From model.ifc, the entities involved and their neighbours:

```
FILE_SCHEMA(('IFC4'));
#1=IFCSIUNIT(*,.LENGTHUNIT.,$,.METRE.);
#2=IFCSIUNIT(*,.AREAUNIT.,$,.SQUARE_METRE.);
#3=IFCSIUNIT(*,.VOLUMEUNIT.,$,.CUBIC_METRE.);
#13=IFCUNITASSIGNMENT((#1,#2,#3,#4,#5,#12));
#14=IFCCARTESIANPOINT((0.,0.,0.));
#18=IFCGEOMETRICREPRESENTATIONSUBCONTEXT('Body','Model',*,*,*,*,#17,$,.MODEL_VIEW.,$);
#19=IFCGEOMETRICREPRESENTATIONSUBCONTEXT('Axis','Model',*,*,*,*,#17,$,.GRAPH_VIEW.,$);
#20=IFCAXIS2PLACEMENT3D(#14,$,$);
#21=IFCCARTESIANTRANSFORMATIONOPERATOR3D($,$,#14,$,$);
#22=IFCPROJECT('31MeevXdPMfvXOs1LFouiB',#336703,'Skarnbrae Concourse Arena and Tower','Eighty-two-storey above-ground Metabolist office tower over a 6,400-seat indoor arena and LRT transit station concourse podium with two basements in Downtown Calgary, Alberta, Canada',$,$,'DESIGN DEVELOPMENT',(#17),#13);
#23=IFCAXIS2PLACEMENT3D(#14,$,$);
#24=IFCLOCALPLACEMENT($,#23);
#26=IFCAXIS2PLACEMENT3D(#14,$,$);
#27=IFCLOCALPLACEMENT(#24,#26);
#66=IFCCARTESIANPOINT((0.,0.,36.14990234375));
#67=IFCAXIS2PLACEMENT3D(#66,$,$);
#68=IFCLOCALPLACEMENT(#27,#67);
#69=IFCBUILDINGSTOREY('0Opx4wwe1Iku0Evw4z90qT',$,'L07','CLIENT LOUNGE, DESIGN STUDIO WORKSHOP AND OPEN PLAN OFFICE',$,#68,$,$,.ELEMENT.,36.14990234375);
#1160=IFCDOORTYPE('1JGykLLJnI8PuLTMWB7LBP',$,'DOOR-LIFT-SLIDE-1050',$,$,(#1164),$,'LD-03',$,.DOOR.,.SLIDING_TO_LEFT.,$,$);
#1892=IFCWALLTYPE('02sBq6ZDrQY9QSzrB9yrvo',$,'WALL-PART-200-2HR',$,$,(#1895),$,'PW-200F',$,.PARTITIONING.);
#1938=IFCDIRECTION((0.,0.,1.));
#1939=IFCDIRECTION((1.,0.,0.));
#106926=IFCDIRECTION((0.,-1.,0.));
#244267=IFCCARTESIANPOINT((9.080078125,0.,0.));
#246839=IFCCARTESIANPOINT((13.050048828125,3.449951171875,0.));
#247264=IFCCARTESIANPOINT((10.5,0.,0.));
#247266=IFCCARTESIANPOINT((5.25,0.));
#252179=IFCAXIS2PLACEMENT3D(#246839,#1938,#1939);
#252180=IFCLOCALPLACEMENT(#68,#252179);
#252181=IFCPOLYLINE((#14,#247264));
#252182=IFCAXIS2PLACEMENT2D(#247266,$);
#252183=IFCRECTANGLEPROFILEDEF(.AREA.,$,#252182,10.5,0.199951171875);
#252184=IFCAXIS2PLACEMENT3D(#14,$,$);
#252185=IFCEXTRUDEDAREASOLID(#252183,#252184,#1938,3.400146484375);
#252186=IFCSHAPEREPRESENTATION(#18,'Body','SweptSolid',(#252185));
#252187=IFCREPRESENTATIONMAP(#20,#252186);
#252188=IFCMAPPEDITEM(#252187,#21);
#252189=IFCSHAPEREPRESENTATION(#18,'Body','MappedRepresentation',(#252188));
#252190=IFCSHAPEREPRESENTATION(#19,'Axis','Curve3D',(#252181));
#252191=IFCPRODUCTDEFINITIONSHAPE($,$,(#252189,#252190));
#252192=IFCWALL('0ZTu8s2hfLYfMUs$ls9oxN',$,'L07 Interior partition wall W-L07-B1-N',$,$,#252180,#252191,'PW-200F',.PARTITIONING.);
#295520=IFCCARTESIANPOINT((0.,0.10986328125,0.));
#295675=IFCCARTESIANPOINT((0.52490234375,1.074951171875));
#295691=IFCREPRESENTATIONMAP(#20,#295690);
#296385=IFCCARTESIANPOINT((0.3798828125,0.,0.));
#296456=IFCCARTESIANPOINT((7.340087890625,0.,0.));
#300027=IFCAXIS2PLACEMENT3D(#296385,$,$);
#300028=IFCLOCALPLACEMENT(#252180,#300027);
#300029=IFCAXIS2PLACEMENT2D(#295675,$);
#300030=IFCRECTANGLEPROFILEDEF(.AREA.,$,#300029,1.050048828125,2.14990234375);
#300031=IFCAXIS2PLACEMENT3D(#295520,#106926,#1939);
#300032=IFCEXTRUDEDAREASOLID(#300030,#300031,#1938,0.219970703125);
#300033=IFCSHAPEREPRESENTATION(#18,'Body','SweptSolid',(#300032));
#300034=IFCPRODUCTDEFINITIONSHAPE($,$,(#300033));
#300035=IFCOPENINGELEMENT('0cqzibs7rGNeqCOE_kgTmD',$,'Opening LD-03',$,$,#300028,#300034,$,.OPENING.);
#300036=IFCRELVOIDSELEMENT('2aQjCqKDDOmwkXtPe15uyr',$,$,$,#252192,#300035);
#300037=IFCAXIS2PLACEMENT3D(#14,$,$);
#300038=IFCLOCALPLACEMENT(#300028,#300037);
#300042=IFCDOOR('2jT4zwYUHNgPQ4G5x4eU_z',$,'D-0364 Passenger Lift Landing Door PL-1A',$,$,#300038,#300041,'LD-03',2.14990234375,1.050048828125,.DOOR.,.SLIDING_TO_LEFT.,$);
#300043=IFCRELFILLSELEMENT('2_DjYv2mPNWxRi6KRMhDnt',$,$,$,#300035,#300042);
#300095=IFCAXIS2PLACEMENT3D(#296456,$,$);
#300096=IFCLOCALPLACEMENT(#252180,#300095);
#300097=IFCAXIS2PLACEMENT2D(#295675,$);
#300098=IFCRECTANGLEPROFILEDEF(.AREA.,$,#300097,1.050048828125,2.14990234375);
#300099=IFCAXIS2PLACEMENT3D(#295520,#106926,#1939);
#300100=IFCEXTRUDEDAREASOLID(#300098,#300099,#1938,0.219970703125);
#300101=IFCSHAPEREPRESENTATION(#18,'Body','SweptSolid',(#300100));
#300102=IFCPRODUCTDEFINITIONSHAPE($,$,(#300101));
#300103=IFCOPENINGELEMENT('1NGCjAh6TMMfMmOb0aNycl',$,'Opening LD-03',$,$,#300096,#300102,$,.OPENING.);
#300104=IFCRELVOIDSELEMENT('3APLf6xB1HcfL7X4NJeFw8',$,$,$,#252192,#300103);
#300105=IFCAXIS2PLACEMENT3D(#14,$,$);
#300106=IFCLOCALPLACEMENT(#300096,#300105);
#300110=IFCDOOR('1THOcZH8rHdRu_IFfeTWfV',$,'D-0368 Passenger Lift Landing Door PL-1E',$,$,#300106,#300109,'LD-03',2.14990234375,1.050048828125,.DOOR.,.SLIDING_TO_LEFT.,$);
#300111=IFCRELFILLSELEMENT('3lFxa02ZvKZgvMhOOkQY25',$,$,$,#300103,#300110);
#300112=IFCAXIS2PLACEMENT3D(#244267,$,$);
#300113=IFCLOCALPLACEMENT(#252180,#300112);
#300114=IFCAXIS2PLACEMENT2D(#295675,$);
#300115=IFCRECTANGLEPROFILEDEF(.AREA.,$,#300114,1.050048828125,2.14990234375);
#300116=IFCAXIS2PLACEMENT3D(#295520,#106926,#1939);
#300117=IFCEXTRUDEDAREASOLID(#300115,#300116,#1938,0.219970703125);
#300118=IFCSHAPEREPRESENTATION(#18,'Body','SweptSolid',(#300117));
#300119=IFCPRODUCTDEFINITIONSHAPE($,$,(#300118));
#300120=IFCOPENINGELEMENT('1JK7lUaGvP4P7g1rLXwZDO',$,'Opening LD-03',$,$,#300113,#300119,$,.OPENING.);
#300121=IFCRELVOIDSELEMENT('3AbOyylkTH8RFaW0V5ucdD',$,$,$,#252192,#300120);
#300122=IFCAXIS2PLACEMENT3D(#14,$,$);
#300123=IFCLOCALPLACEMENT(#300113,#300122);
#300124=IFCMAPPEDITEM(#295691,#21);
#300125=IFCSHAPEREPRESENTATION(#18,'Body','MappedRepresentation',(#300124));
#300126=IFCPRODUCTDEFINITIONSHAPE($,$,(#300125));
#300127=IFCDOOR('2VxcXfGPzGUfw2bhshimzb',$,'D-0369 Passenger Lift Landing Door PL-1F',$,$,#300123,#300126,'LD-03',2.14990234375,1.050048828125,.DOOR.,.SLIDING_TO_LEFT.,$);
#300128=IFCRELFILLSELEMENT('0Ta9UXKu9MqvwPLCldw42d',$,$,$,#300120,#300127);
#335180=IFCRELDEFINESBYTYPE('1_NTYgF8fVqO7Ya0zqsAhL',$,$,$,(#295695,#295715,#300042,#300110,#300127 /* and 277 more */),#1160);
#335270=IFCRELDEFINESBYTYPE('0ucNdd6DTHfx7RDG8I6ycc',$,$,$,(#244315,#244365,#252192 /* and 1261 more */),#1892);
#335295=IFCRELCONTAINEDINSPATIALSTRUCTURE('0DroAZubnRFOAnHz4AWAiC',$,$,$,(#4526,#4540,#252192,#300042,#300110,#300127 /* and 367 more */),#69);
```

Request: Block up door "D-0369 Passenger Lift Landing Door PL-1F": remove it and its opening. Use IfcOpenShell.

```python
import ifcopenshell
import ifcopenshell.api.feature
import ifcopenshell.api.root
import ifcopenshell.geom
import ifcopenshell.util.shape

model = ifcopenshell.open("model.ifc")
settings = ifcopenshell.geom.settings()


def volume(element):
    """Net volume in cubic metres, openings subtracted."""
    shape = ifcopenshell.geom.create_shape(settings, element)
    return ifcopenshell.util.shape.get_volume(shape.geometry)


door = model.by_guid("2VxcXfGPzGUfw2bhshimzb")
opening = door.FillsVoids[0].RelatingOpeningElement
wall = opening.VoidsElements[0].RelatingBuildingElement
before = volume(wall)

ifcopenshell.api.root.remove_product(model, product=door)
ifcopenshell.api.feature.remove_feature(model, feature=opening)

after = volume(wall)

print(f"wall volume {before:.3f} -> {after:.3f} m3")

model.write("model_updated.ifc")
```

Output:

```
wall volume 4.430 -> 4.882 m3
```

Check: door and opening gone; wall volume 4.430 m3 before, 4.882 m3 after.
